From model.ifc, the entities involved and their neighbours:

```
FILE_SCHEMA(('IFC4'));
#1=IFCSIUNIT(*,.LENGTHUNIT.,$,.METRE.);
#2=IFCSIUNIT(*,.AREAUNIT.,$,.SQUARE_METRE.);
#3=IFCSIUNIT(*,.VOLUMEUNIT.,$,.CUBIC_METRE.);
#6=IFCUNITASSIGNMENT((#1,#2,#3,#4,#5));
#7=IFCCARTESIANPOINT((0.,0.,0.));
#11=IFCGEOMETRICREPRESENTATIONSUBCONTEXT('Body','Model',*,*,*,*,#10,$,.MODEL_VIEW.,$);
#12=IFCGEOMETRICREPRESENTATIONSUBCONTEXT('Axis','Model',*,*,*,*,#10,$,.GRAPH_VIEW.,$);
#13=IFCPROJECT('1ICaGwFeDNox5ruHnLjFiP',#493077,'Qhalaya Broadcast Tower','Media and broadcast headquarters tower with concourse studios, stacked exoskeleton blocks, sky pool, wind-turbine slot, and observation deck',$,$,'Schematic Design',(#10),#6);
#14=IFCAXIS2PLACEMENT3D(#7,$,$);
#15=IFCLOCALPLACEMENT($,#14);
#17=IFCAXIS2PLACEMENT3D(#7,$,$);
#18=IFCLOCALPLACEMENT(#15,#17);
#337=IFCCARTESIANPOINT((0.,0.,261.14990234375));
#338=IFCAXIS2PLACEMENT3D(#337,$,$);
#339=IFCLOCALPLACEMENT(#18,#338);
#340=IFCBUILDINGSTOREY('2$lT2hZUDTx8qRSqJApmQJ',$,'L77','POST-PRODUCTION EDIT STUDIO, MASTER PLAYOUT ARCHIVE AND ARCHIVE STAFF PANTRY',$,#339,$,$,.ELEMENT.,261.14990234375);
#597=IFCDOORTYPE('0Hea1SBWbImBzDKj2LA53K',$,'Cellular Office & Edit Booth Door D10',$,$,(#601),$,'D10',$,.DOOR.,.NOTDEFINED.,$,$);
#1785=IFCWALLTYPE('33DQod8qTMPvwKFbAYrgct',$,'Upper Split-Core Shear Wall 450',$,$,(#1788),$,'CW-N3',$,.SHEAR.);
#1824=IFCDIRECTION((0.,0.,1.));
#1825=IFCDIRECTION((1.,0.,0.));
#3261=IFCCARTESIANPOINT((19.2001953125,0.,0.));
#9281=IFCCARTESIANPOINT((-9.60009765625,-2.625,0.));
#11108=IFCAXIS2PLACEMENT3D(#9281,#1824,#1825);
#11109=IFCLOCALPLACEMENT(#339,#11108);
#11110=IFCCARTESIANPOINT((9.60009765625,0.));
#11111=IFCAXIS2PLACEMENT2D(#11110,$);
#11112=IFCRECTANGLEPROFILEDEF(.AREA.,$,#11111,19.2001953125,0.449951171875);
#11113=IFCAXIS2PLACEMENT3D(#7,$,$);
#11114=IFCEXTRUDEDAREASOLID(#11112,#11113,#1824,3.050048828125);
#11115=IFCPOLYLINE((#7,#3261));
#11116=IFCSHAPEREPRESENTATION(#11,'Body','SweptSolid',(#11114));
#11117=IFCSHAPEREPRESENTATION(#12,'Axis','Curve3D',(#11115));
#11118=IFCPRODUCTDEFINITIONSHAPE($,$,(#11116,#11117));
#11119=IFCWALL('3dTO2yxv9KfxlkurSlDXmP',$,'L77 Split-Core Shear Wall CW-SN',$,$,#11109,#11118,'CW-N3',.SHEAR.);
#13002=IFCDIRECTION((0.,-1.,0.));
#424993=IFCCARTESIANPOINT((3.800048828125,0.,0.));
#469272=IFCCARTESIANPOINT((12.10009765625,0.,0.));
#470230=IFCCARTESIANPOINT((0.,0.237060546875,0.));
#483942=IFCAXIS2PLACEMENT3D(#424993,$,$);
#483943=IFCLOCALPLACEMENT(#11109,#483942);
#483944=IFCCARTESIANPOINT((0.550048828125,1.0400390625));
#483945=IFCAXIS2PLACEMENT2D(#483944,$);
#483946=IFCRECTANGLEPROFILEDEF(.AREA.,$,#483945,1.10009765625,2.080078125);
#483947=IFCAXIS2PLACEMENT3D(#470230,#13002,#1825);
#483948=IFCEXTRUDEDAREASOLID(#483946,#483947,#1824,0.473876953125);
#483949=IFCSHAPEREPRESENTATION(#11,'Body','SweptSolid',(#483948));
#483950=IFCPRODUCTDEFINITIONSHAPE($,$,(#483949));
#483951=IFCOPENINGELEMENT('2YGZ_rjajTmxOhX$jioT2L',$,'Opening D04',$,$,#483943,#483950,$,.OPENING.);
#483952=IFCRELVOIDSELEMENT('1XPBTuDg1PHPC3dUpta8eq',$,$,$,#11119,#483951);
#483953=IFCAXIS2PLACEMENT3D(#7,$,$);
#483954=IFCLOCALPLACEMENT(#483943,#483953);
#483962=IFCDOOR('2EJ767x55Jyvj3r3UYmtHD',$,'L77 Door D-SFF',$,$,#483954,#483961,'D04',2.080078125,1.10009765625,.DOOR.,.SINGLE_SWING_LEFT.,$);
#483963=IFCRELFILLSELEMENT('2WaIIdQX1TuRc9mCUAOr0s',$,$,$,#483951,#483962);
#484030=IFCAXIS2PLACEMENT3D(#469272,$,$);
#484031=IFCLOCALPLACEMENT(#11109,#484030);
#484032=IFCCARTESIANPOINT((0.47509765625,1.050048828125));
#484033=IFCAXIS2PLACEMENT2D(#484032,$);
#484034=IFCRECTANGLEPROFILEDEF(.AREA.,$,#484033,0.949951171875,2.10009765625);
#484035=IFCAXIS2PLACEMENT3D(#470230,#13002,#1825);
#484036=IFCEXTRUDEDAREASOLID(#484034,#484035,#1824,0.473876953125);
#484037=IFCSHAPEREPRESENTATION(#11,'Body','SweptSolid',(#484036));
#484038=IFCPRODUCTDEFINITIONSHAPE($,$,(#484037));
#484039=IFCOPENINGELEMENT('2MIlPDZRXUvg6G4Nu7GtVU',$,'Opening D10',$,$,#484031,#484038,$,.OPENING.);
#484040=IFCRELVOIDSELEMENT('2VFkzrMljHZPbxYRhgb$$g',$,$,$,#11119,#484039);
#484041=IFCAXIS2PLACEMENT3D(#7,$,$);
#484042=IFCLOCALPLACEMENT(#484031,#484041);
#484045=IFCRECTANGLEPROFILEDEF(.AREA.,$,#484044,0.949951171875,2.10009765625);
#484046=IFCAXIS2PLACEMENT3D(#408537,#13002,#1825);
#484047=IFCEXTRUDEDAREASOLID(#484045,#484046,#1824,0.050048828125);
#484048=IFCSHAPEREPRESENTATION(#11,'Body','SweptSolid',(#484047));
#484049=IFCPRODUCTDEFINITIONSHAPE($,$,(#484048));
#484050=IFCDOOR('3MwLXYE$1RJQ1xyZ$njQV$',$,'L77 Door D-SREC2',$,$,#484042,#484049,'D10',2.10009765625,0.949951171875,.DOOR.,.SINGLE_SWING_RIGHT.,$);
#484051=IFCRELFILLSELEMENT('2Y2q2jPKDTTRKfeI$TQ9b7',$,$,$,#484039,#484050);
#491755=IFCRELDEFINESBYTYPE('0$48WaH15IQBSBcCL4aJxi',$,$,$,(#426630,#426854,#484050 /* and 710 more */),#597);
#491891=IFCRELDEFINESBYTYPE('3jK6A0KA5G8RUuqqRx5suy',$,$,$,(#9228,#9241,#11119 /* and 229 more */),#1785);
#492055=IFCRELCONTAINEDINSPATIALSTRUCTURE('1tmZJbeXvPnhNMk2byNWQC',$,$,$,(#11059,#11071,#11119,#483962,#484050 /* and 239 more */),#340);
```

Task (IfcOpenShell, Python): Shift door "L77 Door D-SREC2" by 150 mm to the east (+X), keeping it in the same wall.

```python
import ifcopenshell
import ifcopenshell.api.geometry
import ifcopenshell.util.placement
import ifcopenshell.util.unit

model = ifcopenshell.open("model.ifc")
unit_scale = ifcopenshell.util.unit.calculate_unit_scale(model)

door = model.by_guid("3MwLXYE$1RJQ1xyZ$njQV$")
opening = door.FillsVoids[0].RelatingOpeningElement
wall = opening.VoidsElements[0].RelatingBuildingElement

wall_matrix = ifcopenshell.util.placement.get_local_placement(wall.ObjectPlacement)
shift = wall_matrix[:3, 0] * 0.15 / unit_scale
before = ifcopenshell.util.placement.get_local_placement(door.ObjectPlacement)[:3, 3].copy()

# The door is placed relative to its opening, so it follows when the opening moves.
matrix = ifcopenshell.util.placement.get_local_placement(opening.ObjectPlacement)
matrix[:3, 3] += shift
ifcopenshell.api.geometry.edit_object_placement(
    model, product=opening, matrix=matrix, is_si=False, should_transform_children=True
)

after = ifcopenshell.util.placement.get_local_placement(door.ObjectPlacement)[:3, 3]
print("door moved by", (after - before).round(3) + 0.0)

model.write("model_v2.ifc")
```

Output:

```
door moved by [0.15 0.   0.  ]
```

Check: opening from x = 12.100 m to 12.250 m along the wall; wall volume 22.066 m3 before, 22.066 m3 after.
